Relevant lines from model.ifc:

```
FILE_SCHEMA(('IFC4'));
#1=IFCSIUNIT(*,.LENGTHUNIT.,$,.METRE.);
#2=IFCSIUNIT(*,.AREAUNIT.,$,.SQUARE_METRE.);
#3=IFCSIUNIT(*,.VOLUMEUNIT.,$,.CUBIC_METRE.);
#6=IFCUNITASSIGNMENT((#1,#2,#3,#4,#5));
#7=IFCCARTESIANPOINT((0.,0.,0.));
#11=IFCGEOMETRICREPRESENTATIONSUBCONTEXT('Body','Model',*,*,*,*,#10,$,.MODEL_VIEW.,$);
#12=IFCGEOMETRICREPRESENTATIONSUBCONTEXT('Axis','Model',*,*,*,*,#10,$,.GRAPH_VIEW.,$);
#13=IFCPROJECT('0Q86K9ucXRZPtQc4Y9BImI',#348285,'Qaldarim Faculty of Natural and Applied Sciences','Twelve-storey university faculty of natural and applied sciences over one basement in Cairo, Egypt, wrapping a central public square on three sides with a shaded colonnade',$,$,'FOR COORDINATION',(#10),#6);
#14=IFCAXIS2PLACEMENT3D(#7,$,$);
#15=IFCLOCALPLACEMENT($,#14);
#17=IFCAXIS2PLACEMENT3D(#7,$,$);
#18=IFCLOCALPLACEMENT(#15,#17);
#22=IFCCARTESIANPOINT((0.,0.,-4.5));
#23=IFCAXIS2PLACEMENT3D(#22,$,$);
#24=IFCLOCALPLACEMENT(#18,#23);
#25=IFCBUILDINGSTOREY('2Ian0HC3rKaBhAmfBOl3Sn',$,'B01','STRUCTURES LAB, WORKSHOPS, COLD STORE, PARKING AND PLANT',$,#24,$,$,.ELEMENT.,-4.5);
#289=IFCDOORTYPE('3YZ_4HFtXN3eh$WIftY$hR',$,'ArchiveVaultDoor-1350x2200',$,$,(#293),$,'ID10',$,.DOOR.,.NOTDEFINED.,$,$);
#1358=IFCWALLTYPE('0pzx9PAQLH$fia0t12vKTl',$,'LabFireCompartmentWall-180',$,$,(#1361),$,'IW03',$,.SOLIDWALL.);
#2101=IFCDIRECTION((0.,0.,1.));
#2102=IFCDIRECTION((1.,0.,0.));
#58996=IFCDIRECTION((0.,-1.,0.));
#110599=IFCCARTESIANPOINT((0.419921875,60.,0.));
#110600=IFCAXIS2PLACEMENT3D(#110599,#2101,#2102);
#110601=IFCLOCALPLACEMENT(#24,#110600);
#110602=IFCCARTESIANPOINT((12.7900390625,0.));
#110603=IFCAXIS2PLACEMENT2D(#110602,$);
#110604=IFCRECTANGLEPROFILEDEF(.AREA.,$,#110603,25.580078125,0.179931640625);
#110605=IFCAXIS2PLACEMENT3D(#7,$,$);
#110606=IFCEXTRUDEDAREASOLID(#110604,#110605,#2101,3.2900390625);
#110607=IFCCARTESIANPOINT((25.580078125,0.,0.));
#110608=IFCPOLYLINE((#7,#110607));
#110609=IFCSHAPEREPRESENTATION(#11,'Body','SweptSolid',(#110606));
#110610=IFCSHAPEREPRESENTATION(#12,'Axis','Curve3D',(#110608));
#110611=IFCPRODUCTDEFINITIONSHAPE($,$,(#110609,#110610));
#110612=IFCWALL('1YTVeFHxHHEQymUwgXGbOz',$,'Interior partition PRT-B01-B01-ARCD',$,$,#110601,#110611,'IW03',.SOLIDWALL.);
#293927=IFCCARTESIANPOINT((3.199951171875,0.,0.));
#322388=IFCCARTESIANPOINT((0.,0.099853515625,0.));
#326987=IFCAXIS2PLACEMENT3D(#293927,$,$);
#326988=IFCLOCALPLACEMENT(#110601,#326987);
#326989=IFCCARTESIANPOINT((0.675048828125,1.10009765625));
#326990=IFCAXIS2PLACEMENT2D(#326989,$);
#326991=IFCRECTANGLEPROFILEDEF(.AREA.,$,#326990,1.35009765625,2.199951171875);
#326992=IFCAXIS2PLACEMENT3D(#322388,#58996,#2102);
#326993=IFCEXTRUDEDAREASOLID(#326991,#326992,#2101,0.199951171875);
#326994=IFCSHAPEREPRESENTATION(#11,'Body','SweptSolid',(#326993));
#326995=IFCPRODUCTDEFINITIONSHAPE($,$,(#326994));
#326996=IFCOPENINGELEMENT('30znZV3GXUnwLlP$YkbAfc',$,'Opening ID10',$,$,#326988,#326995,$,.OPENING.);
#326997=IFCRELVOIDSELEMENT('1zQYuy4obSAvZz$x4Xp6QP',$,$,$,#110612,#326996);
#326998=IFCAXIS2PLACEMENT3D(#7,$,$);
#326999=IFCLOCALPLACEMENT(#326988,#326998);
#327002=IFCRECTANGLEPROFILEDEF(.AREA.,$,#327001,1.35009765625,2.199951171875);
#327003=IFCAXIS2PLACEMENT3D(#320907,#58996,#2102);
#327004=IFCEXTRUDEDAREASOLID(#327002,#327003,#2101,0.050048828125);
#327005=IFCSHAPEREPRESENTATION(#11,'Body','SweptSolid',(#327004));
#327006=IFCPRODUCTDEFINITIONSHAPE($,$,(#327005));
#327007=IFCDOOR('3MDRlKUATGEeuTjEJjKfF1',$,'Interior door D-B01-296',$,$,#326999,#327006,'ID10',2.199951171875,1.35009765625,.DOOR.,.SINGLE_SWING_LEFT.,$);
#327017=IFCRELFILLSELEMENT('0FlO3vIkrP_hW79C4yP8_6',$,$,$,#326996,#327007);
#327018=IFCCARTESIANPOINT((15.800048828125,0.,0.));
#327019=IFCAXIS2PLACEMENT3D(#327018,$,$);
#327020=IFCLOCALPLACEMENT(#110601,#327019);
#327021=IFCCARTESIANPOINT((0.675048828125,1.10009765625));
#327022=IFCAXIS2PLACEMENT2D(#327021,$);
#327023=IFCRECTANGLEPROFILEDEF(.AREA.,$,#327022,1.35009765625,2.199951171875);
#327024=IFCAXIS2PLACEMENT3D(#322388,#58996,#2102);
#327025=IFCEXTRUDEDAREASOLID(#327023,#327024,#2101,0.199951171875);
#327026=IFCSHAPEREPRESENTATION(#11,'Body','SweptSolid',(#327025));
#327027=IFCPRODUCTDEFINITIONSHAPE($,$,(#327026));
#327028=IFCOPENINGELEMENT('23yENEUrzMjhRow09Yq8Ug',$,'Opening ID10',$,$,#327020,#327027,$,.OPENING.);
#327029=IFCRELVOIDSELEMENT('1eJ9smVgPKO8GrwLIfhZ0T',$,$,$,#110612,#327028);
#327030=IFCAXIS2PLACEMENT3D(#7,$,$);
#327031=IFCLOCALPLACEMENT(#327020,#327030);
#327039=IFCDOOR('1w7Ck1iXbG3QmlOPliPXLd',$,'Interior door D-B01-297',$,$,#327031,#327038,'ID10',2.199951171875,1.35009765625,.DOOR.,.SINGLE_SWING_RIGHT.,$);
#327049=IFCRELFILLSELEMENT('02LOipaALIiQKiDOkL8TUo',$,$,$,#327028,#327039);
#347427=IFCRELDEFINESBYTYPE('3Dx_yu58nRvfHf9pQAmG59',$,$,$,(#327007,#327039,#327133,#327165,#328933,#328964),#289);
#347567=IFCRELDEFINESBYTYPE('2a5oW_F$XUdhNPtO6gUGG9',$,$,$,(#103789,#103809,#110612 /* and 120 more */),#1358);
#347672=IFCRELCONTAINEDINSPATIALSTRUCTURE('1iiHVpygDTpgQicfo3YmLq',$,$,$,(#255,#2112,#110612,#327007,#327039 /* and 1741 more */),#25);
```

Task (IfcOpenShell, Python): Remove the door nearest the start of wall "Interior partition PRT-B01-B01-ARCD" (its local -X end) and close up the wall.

```python
import ifcopenshell
import ifcopenshell.api.feature
import ifcopenshell.api.root
import ifcopenshell.geom
import ifcopenshell.util.shape

model = ifcopenshell.open("model.ifc")
settings = ifcopenshell.geom.settings()


def volume(element):
    """Net volume in cubic metres, openings subtracted."""
    shape = ifcopenshell.geom.create_shape(settings, element)
    return ifcopenshell.util.shape.get_volume(shape.geometry)


door = model.by_id(327007)
opening = door.FillsVoids[0].RelatingOpeningElement
wall = opening.VoidsElements[0].RelatingBuildingElement
before = volume(wall)

ifcopenshell.api.root.remove_product(model, product=door)
ifcopenshell.api.feature.remove_feature(model, feature=opening)

after = volume(wall)

print(f"wall volume {before:.3f} -> {after:.3f} m3")

model.write("model_rev.ifc")
```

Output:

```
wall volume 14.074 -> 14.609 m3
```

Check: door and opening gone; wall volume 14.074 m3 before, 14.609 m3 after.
